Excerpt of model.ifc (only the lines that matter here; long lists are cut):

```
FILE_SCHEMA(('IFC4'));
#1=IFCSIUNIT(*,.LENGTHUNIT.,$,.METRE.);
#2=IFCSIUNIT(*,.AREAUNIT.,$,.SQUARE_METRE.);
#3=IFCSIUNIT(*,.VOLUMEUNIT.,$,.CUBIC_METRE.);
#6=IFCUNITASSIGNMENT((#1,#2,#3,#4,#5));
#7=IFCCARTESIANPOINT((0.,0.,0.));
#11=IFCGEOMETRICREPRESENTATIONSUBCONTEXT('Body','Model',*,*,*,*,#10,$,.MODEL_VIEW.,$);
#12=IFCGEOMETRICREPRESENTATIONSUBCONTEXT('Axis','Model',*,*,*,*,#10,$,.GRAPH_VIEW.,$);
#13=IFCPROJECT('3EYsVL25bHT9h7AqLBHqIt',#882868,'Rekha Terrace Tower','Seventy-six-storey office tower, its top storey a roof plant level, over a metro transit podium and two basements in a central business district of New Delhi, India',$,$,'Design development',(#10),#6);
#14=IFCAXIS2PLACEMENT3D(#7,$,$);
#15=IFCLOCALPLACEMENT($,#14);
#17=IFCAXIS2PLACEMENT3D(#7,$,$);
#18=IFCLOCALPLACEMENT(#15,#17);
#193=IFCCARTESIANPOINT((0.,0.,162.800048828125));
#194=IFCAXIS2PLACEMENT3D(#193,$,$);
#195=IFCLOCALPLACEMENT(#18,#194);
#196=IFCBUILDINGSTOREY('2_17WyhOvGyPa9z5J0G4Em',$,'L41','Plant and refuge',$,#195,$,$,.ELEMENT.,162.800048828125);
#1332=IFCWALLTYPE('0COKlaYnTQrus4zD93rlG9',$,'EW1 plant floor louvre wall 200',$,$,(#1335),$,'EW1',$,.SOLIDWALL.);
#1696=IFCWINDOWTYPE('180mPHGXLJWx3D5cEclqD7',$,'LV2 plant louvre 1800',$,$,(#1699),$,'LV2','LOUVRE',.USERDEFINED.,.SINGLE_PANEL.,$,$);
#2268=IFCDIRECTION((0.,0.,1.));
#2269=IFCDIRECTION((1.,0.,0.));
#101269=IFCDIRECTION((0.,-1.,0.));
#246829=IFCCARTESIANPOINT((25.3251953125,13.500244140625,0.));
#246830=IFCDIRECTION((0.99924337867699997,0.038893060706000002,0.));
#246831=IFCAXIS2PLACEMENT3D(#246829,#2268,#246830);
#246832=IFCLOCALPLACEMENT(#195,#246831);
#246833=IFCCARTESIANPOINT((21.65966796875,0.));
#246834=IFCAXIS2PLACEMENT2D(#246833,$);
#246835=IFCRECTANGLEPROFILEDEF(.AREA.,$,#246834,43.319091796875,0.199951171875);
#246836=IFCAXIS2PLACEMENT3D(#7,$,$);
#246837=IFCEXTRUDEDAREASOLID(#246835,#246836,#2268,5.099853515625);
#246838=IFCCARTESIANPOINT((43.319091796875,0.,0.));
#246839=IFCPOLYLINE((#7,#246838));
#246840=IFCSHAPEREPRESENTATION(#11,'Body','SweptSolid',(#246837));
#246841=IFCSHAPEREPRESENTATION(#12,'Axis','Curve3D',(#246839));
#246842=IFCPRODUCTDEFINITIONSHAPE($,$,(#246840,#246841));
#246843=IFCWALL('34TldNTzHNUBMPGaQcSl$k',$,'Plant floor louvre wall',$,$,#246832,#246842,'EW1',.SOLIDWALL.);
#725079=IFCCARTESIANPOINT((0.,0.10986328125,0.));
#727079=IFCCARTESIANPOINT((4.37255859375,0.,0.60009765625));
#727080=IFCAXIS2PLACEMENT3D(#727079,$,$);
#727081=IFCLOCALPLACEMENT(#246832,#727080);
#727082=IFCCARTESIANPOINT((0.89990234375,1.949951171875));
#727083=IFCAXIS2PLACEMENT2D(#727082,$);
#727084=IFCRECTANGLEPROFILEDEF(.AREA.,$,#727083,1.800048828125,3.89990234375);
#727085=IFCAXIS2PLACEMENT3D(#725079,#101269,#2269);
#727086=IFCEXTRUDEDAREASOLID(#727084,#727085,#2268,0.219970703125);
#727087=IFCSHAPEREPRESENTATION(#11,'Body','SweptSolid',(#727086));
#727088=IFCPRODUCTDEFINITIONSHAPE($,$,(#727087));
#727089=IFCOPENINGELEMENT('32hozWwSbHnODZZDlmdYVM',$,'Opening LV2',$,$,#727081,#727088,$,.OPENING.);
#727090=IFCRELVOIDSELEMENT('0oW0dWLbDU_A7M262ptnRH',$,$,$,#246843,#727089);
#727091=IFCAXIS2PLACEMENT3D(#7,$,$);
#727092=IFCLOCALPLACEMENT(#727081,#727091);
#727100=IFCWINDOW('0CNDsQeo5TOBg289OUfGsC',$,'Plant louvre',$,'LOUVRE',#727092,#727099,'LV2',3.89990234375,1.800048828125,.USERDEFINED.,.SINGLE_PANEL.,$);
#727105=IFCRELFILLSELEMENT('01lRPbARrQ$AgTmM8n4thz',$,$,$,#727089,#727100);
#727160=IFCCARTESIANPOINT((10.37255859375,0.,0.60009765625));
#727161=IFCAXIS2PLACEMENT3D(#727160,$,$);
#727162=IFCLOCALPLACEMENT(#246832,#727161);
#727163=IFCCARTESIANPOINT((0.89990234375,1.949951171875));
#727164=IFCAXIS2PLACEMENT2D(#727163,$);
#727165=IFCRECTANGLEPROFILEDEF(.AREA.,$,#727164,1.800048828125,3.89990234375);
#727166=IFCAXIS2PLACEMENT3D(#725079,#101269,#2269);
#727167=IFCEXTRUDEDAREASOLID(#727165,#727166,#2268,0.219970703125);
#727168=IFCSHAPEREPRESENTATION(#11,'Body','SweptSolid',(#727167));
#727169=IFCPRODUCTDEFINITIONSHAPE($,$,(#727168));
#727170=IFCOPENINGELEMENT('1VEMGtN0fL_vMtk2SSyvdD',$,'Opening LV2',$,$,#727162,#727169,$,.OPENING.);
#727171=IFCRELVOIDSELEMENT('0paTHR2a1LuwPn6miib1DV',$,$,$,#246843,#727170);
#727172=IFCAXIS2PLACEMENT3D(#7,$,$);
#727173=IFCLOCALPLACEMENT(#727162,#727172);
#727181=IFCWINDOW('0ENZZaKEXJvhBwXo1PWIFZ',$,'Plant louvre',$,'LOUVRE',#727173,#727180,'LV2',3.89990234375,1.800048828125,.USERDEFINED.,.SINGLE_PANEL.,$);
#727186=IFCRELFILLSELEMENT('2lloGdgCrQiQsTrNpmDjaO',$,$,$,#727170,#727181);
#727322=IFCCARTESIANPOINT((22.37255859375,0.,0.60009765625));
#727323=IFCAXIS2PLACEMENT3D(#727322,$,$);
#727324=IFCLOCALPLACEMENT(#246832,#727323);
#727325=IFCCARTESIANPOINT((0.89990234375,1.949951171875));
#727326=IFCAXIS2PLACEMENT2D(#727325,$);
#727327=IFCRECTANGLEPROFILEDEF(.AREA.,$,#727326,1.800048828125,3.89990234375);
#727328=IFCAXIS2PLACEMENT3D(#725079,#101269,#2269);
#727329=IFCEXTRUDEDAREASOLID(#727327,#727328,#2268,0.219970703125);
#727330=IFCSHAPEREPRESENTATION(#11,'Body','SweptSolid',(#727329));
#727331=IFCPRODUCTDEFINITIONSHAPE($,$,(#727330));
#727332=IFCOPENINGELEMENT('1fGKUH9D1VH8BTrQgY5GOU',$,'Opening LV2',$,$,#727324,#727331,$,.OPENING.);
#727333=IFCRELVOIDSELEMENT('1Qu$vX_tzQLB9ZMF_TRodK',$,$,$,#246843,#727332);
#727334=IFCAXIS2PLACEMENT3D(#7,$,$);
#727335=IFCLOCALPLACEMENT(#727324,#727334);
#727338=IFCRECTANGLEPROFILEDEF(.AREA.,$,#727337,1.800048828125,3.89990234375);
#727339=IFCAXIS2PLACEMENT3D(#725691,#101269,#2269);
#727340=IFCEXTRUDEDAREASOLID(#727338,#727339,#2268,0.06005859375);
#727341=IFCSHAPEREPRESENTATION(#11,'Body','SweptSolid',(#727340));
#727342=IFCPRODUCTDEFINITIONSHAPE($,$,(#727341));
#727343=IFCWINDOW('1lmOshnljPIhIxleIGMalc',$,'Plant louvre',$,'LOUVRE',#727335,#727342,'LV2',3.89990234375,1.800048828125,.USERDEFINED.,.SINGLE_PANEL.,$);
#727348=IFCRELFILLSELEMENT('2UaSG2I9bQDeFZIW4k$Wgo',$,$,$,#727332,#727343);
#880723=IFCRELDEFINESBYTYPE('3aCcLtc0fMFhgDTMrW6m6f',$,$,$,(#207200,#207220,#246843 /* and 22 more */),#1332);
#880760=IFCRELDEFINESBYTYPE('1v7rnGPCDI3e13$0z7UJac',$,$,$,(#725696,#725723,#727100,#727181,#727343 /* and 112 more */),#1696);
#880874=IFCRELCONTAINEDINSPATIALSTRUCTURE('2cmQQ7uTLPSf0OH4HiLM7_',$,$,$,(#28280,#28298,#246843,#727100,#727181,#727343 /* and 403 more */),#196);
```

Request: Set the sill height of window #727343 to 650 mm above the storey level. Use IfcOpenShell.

```python
import numpy as np
import ifcopenshell
import ifcopenshell.api.geometry
import ifcopenshell.geom
import ifcopenshell.util.element
import ifcopenshell.util.placement
import ifcopenshell.util.shape
import ifcopenshell.util.unit

model = ifcopenshell.open("model.ifc")
unit_scale = ifcopenshell.util.unit.calculate_unit_scale(model)

window = model.by_id(727343)
opening = window.FillsVoids[0].RelatingOpeningElement
storey = ifcopenshell.util.element.get_container(window, ifc_class="IfcBuildingStorey")
level = ifcopenshell.util.placement.get_local_placement(storey.ObjectPlacement)[2, 3]

# The opening's origin need not be at the sill, so measure its lowest point.
shape = ifcopenshell.geom.create_shape(ifcopenshell.geom.settings(), opening)
bottom = ifcopenshell.util.shape.get_shape_bottom_elevation(shape, shape.geometry) / unit_scale
dz = level + 0.65 / unit_scale - bottom

shift = np.array([0.0, 0.0, dz])
# The window is placed relative to its opening, so it follows when the opening moves.
matrix = ifcopenshell.util.placement.get_local_placement(opening.ObjectPlacement)
matrix[:3, 3] += shift
ifcopenshell.api.geometry.edit_object_placement(
    model, product=opening, matrix=matrix, is_si=False, should_transform_children=True
)

print(f"moved by {dz * unit_scale:+.3f} m")

model.write("model_edited.ifc")
```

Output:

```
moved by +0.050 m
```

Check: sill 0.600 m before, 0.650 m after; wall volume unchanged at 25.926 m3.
